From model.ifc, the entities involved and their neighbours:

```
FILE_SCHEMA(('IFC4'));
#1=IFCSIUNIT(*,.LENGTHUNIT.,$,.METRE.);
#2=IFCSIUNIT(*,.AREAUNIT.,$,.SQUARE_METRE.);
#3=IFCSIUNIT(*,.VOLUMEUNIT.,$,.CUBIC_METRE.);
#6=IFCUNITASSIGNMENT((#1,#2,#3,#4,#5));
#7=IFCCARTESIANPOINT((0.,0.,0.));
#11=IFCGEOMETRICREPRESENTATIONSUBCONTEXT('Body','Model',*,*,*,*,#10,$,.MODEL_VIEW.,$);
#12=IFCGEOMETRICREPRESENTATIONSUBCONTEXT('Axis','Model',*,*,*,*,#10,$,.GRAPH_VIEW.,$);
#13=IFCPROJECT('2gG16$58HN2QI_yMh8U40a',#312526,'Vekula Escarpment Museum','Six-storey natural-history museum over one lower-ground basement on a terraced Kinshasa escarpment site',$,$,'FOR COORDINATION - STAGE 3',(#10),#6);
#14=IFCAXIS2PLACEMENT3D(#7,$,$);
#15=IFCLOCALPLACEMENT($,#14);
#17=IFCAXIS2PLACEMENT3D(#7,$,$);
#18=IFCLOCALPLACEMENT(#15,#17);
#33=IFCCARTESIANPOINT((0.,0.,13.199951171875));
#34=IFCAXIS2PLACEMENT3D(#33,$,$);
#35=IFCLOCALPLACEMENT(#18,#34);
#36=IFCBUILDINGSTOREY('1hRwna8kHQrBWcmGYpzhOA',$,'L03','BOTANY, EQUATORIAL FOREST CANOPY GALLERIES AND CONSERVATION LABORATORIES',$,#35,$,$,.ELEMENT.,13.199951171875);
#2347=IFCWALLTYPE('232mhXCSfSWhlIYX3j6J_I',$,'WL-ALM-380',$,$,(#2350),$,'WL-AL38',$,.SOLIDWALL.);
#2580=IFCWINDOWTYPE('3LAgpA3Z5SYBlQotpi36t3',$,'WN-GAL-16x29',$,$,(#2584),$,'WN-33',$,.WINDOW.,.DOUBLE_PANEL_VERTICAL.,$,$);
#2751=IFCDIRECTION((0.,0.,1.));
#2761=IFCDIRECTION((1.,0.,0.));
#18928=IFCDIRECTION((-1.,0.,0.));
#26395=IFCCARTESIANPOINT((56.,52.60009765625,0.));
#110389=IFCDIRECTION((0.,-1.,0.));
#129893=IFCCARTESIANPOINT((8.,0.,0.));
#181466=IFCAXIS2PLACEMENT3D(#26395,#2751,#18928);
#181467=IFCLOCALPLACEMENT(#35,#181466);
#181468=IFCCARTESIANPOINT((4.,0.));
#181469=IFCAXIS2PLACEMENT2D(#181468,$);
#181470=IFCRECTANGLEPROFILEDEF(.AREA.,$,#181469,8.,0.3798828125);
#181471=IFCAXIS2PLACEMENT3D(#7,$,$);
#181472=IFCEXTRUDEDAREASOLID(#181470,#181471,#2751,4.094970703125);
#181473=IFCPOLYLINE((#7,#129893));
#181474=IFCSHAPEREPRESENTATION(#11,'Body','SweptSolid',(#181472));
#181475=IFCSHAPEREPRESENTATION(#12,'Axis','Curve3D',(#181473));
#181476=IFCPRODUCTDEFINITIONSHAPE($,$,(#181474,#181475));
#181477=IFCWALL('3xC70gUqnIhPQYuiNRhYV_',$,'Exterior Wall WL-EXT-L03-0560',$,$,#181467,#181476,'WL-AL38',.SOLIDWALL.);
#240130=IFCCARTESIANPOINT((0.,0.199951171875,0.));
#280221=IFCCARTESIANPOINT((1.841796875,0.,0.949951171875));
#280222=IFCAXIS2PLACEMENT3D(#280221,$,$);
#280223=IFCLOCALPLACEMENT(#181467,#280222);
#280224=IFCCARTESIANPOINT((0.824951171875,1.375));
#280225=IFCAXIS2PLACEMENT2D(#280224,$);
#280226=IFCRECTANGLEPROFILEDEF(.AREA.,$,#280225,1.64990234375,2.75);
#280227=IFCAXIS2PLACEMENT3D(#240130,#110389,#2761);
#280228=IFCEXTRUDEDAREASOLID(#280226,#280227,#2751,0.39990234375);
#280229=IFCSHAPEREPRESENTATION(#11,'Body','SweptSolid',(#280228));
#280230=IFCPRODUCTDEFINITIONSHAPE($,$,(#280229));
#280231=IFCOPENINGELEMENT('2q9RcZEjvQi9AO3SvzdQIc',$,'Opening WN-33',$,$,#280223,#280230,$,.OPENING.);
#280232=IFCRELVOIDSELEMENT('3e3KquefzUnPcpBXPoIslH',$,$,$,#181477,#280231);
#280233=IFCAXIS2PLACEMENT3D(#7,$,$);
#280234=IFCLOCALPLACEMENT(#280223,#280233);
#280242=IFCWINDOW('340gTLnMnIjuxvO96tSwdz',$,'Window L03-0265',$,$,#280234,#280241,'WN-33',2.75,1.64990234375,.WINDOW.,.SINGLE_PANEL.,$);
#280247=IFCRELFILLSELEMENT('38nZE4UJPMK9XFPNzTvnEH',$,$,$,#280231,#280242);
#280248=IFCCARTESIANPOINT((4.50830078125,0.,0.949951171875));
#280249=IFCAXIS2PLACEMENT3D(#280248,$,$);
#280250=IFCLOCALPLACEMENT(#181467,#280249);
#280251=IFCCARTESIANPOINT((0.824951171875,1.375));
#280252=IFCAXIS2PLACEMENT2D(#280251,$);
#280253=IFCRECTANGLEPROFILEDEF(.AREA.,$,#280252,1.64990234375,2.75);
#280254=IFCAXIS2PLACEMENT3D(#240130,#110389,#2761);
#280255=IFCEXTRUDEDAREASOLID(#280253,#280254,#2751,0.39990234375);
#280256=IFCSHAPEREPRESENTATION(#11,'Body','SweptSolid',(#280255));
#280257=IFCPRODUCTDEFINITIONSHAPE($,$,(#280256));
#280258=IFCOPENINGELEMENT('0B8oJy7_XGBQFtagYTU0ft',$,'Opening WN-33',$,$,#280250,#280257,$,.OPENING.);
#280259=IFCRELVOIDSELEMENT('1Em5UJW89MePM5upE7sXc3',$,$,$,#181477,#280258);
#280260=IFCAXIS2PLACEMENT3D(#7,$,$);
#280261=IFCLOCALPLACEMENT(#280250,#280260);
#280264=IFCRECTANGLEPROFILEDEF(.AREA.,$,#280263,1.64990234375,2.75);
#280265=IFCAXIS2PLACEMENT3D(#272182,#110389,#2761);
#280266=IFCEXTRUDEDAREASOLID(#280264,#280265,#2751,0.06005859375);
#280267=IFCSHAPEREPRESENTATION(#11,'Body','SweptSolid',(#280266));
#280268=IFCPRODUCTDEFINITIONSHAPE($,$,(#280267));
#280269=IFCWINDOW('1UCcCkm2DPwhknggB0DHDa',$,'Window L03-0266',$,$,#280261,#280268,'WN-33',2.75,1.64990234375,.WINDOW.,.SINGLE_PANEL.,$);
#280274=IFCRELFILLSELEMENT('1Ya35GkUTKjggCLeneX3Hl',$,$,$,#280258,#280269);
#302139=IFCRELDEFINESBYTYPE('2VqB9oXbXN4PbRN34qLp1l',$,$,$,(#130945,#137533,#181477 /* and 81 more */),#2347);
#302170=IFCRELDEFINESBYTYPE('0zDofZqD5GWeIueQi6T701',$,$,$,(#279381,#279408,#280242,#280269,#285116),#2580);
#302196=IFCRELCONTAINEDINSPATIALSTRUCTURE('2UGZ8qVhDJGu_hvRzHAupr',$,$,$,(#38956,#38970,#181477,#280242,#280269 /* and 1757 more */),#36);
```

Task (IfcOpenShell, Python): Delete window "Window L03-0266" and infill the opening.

```python
import ifcopenshell
import ifcopenshell.api.feature
import ifcopenshell.api.root
import ifcopenshell.geom
import ifcopenshell.util.shape

model = ifcopenshell.open("model.ifc")
settings = ifcopenshell.geom.settings()


def volume(element):
    """Net volume in cubic metres, openings subtracted."""
    shape = ifcopenshell.geom.create_shape(settings, element)
    return ifcopenshell.util.shape.get_volume(shape.geometry)


window = model.by_guid("1UCcCkm2DPwhknggB0DHDa")
opening = window.FillsVoids[0].RelatingOpeningElement
wall = opening.VoidsElements[0].RelatingBuildingElement
before = volume(wall)

ifcopenshell.api.root.remove_product(model, product=window)
ifcopenshell.api.feature.remove_feature(model, feature=opening)

after = volume(wall)

print(f"wall volume {before:.3f} -> {after:.3f} m3")

model.write("model_edited.ifc")
```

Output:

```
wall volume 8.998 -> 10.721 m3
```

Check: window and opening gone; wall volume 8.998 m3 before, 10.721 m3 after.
